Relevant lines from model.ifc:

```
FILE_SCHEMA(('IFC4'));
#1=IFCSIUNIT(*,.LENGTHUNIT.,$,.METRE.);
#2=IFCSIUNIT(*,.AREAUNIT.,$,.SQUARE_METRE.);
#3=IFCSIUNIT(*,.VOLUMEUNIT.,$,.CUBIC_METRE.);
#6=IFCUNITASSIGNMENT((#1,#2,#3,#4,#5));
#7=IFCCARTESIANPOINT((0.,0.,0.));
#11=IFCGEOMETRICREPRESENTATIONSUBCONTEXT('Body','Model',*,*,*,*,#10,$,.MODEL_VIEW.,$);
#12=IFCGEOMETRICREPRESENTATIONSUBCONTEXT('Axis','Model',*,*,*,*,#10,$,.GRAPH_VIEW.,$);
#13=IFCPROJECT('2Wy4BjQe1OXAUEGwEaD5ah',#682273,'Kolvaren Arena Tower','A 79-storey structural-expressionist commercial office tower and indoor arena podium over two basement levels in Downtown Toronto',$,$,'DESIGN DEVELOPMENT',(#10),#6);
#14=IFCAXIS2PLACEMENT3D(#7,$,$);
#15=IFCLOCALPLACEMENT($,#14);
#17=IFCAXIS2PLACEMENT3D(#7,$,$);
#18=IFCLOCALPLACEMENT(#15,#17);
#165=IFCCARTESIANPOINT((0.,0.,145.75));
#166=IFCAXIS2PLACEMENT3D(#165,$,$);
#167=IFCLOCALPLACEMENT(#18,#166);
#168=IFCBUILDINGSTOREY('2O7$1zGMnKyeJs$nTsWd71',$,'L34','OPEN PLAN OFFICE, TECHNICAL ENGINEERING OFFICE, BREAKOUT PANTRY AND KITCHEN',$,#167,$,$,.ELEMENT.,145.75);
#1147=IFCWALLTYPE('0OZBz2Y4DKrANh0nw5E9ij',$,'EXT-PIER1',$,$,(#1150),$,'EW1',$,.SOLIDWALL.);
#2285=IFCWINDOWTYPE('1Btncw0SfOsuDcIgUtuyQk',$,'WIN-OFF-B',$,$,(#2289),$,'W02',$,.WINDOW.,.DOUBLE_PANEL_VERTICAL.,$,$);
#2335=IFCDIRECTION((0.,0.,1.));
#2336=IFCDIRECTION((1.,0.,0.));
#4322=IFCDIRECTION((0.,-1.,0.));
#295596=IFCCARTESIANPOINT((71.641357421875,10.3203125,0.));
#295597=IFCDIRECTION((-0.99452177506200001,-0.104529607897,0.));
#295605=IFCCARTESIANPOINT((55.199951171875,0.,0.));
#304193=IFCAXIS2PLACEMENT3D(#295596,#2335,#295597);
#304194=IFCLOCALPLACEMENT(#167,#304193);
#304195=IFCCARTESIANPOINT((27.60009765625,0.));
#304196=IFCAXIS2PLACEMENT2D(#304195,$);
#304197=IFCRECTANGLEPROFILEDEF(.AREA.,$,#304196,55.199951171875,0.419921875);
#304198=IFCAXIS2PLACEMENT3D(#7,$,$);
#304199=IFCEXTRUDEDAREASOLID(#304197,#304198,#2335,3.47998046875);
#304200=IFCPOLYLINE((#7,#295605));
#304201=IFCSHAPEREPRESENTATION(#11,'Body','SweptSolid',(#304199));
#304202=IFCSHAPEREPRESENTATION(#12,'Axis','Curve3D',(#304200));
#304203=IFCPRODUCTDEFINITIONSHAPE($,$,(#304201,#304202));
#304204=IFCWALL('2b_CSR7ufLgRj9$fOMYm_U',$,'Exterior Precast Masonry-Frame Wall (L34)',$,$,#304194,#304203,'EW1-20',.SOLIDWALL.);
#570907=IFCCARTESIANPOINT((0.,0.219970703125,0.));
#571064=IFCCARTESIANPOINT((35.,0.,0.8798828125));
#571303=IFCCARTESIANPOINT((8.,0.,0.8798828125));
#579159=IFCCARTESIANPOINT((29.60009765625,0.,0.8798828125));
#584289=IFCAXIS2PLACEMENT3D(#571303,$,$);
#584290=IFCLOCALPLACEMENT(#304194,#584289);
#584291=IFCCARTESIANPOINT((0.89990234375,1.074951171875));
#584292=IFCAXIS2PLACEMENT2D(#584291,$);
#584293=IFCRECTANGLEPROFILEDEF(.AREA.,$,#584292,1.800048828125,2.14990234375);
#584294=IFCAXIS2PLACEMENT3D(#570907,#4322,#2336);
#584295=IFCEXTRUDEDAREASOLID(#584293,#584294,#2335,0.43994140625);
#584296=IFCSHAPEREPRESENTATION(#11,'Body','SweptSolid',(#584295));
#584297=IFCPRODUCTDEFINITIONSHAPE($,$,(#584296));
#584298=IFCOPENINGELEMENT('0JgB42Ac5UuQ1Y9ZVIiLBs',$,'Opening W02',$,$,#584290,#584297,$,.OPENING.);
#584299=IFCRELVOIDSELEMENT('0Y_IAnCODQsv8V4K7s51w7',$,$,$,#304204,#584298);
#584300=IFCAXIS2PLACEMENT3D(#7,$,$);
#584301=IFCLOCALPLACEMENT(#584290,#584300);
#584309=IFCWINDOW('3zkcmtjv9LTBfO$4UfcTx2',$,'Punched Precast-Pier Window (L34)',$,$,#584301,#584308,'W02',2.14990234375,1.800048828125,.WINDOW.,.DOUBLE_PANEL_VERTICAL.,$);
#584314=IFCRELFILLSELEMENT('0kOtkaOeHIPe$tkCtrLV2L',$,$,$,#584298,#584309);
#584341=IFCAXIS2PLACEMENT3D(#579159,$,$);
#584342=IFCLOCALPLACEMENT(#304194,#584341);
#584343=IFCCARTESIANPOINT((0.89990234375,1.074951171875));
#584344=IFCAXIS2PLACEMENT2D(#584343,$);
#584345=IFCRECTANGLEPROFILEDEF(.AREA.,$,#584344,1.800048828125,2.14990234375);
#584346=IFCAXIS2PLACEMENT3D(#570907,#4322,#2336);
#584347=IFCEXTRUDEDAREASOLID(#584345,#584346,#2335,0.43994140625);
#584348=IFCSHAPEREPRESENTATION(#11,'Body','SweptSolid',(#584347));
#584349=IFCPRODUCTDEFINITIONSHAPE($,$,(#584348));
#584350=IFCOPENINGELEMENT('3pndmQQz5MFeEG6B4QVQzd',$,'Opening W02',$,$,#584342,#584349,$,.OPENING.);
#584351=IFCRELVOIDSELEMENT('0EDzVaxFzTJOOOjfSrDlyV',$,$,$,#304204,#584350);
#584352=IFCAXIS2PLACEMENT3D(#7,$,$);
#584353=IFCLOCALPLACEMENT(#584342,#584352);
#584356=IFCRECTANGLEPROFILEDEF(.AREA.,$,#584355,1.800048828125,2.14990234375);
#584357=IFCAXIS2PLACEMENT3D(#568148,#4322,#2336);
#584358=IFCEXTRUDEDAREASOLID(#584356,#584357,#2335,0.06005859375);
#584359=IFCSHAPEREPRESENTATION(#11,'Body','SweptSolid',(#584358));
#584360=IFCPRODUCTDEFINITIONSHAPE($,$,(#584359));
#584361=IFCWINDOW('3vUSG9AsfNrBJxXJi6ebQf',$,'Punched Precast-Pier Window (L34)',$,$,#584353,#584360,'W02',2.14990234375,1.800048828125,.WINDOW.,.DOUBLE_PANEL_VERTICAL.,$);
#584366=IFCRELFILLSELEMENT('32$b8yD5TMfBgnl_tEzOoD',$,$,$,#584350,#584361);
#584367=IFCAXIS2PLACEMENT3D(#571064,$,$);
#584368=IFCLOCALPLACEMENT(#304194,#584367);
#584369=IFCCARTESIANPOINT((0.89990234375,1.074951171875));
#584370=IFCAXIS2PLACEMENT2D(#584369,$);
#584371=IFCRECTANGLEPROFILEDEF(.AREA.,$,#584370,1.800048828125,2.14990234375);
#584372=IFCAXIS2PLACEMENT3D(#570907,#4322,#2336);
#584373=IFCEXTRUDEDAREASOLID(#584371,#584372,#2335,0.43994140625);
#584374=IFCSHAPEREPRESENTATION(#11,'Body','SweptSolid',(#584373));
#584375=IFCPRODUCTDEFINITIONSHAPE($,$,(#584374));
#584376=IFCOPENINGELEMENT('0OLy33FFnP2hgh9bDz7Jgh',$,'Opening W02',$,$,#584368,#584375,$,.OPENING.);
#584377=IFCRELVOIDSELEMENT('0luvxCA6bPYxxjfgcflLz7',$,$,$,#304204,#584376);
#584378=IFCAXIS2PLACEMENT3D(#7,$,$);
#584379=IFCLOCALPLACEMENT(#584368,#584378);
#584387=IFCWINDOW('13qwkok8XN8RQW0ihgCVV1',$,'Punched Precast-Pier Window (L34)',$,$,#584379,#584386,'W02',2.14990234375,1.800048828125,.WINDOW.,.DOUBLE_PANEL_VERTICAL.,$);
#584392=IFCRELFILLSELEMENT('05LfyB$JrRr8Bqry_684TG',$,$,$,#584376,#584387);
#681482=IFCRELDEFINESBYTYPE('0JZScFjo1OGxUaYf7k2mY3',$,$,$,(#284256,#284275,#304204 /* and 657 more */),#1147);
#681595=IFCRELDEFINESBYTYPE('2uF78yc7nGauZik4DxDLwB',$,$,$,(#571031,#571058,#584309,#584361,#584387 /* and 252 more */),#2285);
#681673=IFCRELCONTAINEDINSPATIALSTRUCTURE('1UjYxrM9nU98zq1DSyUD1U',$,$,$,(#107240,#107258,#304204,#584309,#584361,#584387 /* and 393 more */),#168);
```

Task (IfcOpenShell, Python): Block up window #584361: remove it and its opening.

```python
import ifcopenshell
import ifcopenshell.api.feature
import ifcopenshell.api.root
import ifcopenshell.geom
import ifcopenshell.util.shape

model = ifcopenshell.open("model.ifc")
settings = ifcopenshell.geom.settings()


def volume(element):
    """Net volume in cubic metres, openings subtracted."""
    shape = ifcopenshell.geom.create_shape(settings, element)
    return ifcopenshell.util.shape.get_volume(shape.geometry)


window = model.by_guid("3vUSG9AsfNrBJxXJi6ebQf")
opening = window.FillsVoids[0].RelatingOpeningElement
wall = opening.VoidsElements[0].RelatingBuildingElement
before = volume(wall)

ifcopenshell.api.root.remove_product(model, product=window)
ifcopenshell.api.feature.remove_feature(model, feature=opening)

after = volume(wall)

print(f"wall volume {before:.3f} -> {after:.3f} m3")

model.write("model-out.ifc")
```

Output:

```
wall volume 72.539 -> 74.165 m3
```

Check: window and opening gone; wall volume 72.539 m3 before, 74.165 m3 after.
